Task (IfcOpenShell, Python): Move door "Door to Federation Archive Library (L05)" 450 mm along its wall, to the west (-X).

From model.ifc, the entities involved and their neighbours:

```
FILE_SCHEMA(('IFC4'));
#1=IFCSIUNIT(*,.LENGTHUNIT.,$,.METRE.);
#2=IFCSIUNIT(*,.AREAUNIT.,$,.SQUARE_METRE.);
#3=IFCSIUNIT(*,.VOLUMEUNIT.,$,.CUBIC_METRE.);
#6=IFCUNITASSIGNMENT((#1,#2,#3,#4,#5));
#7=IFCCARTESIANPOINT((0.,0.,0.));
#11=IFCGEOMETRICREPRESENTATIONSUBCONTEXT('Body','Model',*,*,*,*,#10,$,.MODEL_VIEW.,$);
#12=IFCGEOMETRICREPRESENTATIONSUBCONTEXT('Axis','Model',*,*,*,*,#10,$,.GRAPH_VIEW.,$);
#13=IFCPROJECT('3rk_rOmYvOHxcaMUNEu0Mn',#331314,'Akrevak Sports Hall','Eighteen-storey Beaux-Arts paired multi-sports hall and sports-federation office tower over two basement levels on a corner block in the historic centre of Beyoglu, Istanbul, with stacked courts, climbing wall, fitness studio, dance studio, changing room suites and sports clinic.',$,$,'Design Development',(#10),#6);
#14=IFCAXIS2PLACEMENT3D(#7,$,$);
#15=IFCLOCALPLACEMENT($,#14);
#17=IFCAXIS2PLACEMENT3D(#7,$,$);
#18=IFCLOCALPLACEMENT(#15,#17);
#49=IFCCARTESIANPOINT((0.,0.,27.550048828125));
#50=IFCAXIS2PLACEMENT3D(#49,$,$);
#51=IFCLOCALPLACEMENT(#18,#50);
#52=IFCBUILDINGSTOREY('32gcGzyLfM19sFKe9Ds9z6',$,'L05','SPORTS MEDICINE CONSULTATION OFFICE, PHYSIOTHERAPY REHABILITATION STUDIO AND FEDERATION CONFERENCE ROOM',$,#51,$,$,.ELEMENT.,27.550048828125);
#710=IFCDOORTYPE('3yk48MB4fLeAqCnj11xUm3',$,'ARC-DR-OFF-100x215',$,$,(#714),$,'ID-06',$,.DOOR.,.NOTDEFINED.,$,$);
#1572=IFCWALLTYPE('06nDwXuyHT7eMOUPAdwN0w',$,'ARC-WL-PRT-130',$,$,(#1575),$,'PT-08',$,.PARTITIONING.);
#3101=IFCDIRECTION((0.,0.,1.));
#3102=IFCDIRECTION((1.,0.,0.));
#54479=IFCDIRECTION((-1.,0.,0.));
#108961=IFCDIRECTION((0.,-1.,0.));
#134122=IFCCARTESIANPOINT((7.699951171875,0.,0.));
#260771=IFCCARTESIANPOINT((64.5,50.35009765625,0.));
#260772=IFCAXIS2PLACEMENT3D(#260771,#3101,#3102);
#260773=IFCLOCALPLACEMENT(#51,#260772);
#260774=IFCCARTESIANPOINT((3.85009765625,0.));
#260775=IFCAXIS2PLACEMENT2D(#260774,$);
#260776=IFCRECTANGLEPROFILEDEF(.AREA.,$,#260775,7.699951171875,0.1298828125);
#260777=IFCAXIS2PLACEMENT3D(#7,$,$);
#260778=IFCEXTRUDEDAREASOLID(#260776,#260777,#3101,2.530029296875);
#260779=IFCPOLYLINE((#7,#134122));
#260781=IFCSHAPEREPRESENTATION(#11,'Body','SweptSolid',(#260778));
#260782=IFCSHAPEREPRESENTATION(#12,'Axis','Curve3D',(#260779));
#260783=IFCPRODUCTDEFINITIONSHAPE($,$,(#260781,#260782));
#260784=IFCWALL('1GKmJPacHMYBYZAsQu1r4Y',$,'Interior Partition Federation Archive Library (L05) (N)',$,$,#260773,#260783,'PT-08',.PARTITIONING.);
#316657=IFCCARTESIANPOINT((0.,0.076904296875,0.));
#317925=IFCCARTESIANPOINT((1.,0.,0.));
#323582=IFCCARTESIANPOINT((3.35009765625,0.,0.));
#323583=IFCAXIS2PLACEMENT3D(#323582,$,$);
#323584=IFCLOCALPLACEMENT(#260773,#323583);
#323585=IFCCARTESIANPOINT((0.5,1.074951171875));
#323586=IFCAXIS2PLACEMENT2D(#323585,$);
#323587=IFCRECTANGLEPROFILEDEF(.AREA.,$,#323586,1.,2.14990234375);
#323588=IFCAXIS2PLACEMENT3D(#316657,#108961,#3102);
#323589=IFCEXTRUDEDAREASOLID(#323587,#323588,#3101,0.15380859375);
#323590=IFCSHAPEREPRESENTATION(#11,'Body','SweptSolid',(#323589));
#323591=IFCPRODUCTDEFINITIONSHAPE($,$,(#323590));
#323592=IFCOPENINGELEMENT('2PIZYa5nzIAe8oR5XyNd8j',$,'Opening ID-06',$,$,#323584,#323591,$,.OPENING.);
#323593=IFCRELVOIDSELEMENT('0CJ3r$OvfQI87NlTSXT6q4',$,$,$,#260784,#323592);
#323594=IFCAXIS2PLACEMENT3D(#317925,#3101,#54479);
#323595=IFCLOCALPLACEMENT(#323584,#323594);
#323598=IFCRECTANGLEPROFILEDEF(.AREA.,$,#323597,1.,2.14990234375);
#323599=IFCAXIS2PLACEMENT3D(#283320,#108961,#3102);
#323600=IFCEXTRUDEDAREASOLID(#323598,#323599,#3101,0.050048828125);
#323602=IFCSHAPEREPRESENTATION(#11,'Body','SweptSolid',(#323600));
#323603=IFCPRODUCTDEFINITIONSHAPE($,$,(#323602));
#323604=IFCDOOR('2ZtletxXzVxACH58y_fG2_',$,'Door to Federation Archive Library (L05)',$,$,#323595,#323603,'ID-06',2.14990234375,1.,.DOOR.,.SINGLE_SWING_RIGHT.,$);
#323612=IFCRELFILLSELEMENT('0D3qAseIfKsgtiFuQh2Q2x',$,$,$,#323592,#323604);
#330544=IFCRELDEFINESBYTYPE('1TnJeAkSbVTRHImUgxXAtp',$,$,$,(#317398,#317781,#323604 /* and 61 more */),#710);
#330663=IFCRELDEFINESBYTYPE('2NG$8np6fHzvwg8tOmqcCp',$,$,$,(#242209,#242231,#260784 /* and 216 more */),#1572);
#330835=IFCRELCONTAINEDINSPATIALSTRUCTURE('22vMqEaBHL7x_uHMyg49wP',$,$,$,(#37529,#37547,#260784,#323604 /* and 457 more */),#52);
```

```python
import ifcopenshell
import ifcopenshell.api.geometry
import ifcopenshell.util.placement

model = ifcopenshell.open("model.ifc")

door = model.by_id(323604)
opening = door.FillsVoids[0].RelatingOpeningElement
wall = opening.VoidsElements[0].RelatingBuildingElement

wall_matrix = ifcopenshell.util.placement.get_local_placement(wall.ObjectPlacement)
shift = wall_matrix[:3, 0] * -0.45
before = ifcopenshell.util.placement.get_local_placement(door.ObjectPlacement)[:3, 3].copy()

# The door is placed relative to its opening, so it follows when the opening moves.
matrix = ifcopenshell.util.placement.get_local_placement(opening.ObjectPlacement)
matrix[:3, 3] += shift
ifcopenshell.api.geometry.edit_object_placement(
    model, product=opening, matrix=matrix, is_si=False, should_transform_children=True
)

after = ifcopenshell.util.placement.get_local_placement(door.ObjectPlacement)[:3, 3]
print("door moved by", (after - before).round(3) + 0.0)

model.write("model-out.ifc")
```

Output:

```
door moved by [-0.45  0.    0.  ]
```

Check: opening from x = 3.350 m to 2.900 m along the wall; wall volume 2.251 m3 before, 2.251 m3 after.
